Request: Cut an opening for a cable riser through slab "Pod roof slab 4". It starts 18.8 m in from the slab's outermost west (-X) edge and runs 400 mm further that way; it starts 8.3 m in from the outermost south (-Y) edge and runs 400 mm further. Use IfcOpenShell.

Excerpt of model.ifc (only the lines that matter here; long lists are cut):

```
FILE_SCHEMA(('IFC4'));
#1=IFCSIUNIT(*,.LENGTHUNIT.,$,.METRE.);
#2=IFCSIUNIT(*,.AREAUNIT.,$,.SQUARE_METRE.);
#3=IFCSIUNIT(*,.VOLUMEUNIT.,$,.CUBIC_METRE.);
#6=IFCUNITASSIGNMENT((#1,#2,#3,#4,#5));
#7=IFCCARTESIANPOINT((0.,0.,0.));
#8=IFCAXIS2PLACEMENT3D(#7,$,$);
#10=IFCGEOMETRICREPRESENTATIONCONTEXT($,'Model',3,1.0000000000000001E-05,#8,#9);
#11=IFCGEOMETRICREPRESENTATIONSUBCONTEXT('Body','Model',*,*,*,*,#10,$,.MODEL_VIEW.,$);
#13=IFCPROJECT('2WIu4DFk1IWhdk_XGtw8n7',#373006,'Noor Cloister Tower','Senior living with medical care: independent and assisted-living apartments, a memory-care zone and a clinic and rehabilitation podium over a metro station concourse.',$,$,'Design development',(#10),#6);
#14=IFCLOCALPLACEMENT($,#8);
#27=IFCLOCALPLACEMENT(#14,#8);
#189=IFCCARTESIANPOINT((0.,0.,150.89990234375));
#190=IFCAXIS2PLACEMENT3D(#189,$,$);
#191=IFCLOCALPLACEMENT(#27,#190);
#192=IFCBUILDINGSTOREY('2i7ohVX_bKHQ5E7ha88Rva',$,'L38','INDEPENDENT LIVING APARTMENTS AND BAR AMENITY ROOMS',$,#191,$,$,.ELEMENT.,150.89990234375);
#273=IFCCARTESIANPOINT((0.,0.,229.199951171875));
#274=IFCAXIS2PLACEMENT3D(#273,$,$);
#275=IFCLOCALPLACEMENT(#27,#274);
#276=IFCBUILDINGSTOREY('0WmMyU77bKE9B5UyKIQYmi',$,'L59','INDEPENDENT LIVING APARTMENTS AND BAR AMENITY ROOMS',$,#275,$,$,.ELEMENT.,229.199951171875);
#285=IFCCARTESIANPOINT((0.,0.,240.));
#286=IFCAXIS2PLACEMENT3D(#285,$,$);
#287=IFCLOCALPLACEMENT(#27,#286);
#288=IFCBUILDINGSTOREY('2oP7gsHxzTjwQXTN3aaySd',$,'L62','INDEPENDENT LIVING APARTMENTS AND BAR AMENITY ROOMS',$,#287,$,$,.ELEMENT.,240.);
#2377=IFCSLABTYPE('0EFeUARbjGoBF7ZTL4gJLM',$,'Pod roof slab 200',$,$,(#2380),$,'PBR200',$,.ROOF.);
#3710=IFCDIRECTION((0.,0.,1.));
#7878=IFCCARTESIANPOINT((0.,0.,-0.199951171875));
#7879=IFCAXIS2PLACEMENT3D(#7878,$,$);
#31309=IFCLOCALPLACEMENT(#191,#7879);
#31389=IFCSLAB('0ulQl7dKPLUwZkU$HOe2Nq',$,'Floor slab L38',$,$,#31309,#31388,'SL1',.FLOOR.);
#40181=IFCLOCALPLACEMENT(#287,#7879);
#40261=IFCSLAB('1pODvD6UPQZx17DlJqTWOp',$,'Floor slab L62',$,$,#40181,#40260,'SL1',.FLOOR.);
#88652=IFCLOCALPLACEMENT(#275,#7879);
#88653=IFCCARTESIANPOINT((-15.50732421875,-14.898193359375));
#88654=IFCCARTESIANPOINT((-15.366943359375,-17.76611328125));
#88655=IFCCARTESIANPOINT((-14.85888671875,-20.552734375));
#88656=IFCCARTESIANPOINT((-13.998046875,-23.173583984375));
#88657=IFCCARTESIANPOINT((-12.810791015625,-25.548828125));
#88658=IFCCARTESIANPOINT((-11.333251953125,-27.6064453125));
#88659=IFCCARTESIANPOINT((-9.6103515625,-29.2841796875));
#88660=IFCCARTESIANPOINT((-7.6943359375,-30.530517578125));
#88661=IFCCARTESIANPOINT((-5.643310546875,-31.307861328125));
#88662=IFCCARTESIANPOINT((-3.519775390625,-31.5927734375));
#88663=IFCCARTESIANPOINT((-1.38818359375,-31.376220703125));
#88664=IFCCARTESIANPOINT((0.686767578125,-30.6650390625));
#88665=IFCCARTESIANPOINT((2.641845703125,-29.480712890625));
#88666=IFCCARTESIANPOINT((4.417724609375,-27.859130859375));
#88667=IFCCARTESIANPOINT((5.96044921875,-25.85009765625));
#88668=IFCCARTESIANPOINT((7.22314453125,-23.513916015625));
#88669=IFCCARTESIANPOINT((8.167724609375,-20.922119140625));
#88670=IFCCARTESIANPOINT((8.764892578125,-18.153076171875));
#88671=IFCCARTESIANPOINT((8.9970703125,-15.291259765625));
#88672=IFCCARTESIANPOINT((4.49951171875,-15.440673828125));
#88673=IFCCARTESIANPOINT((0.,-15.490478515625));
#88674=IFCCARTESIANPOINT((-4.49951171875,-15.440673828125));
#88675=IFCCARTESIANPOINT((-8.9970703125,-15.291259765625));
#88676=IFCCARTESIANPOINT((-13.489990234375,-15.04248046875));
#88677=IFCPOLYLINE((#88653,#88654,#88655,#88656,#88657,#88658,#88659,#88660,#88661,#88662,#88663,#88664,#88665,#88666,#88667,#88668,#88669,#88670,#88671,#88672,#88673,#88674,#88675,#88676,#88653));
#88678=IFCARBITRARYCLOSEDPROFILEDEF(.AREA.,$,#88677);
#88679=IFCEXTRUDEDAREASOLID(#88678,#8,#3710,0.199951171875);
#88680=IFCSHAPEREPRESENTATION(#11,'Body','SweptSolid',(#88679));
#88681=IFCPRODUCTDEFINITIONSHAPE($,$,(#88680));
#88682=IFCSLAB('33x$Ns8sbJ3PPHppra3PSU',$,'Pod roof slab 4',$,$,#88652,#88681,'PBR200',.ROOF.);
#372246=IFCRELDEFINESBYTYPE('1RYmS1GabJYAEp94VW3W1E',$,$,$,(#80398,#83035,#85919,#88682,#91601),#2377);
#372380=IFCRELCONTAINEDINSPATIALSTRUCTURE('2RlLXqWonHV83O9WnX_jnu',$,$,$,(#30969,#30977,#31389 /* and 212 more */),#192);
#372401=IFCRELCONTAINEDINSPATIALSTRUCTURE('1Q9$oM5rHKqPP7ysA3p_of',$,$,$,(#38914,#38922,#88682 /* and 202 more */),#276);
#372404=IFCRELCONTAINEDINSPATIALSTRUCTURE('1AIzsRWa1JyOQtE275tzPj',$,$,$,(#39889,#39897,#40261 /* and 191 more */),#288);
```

```python
import numpy as np
import ifcopenshell
import ifcopenshell.api.feature
import ifcopenshell.api.geometry
import ifcopenshell.api.root
import ifcopenshell.geom
import ifcopenshell.util.placement
import ifcopenshell.util.representation
import ifcopenshell.util.shape
import ifcopenshell.util.unit

model = ifcopenshell.open("model.ifc")
unit_scale = ifcopenshell.util.unit.calculate_unit_scale(model)
settings = ifcopenshell.geom.settings()


def volume(element):
    """Net volume in cubic metres, openings subtracted."""
    shape = ifcopenshell.geom.create_shape(settings, element)
    return ifcopenshell.util.shape.get_volume(shape.geometry)


slab = model.by_guid("33x$Ns8sbJ3PPHppra3PSU")
before = volume(slab)

# Extent in the slab's own axes, in metres. The edges named are its -X and -Y sides.
slab_shape = ifcopenshell.geom.create_shape(settings, slab)
vertices = ifcopenshell.util.shape.get_vertices(slab_shape.geometry)
x_min, y_min, bottom = vertices.min(axis=0)
top = vertices[:, 2].max()

opening = ifcopenshell.api.root.create_entity(model, ifc_class="IfcOpeningElement", name="Cable riser opening", predefined_type="OPENING")
context = ifcopenshell.util.representation.get_context(model, "Model", "Body", "MODEL_VIEW")
width, depth = 0.4, 0.4
outline = [(0.0, 0.0), (width, 0.0), (width, depth), (0.0, depth), (0.0, 0.0)]
# Overshoot both faces by 50 mm so the cut is clean.
shape = ifcopenshell.api.geometry.add_slab_representation(
    model, context=context, depth=top - bottom + 0.1, polyline=outline
)
ifcopenshell.api.geometry.assign_representation(model, product=opening, representation=shape)

matrix = ifcopenshell.util.placement.get_local_placement(slab.ObjectPlacement)
matrix[:, 3] = matrix @ np.append(np.array([x_min + 18.8, y_min + 8.3, bottom - 0.05]) / unit_scale, 1.0)
ifcopenshell.api.geometry.edit_object_placement(model, product=opening, matrix=matrix, is_si=False)
ifcopenshell.api.feature.add_feature(model, feature=opening, element=slab)

after = volume(slab)

print(f"slab volume {before:.3f} -> {after:.3f} m3")

model.write("model-out.ifc")
```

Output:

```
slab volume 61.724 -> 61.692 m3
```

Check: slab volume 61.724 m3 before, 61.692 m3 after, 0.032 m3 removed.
